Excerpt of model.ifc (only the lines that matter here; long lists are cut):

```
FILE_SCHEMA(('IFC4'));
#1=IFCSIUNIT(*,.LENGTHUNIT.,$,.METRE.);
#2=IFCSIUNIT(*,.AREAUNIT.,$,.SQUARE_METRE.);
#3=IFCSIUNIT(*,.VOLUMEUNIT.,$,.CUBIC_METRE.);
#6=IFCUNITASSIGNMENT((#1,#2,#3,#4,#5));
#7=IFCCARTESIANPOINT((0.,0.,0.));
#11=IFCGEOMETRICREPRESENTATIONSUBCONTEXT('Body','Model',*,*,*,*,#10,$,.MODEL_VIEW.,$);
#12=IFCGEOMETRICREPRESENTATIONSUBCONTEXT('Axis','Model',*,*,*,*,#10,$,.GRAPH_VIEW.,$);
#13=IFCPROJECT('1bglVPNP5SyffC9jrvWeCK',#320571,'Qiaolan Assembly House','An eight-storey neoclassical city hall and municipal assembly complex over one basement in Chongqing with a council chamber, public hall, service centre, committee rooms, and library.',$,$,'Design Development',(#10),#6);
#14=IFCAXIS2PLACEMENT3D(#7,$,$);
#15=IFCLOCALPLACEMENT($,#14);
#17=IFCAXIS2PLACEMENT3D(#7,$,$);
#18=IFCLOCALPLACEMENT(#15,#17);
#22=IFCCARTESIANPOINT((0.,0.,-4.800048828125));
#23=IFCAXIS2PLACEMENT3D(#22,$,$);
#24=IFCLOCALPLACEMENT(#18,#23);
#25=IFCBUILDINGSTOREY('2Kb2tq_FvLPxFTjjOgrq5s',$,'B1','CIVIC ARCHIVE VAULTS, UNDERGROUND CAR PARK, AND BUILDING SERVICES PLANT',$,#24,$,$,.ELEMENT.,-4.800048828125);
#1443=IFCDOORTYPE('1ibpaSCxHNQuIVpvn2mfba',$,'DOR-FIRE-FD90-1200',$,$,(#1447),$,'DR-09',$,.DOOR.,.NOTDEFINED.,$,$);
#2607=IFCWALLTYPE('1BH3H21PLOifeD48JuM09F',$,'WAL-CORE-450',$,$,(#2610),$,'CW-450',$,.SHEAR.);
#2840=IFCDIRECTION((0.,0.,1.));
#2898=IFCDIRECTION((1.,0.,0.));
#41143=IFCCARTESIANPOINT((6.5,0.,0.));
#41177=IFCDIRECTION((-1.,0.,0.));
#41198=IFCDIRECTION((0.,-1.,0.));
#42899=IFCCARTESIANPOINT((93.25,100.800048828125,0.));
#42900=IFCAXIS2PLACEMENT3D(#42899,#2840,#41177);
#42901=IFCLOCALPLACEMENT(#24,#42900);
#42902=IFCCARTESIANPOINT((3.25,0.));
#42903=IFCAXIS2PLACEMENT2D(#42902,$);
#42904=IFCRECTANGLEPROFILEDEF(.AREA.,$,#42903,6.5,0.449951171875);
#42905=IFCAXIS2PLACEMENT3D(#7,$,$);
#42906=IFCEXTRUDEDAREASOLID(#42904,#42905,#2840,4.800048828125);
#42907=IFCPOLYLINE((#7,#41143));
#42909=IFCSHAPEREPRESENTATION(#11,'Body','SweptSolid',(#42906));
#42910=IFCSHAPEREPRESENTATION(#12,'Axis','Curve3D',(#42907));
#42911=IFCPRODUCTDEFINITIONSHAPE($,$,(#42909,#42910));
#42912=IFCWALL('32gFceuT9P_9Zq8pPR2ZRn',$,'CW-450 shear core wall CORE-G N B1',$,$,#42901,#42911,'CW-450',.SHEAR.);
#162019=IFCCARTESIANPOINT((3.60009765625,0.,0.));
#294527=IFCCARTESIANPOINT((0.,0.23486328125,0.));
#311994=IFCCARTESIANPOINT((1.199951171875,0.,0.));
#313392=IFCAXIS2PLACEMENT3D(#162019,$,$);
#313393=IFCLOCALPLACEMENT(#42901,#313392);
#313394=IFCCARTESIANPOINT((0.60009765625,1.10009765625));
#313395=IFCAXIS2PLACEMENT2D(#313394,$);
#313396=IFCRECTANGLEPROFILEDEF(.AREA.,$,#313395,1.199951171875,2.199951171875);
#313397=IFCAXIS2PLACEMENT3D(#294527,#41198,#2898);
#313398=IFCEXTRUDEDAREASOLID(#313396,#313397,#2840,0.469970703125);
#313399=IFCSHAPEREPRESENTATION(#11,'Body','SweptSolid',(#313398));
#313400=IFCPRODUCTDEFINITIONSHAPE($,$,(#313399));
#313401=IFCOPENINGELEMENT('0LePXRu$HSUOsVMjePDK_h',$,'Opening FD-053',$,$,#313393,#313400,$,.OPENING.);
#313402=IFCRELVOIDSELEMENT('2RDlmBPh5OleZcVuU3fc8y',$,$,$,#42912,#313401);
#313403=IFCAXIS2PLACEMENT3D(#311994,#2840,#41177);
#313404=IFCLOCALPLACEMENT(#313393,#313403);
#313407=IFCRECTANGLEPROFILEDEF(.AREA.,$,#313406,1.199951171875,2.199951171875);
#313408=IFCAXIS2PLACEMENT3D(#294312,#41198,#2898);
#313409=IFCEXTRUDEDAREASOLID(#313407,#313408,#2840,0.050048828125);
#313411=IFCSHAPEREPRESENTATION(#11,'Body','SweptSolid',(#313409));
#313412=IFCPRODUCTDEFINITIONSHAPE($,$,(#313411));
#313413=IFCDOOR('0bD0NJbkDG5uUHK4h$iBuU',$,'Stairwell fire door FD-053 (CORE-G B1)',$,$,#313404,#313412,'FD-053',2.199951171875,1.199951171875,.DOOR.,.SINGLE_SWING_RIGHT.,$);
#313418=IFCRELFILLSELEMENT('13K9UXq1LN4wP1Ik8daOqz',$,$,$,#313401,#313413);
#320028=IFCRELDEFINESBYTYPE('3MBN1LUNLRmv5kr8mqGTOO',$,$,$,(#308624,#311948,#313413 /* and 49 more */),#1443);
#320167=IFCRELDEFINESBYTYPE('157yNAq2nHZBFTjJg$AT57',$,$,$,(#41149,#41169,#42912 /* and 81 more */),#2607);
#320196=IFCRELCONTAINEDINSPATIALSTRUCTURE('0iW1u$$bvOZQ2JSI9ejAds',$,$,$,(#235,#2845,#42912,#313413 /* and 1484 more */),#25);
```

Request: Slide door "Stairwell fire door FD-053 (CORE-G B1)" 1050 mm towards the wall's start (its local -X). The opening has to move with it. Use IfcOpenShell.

```python
import ifcopenshell
import ifcopenshell.api.geometry
import ifcopenshell.util.placement

model = ifcopenshell.open("model.ifc")

door = model.by_guid("0bD0NJbkDG5uUHK4h$iBuU")
opening = door.FillsVoids[0].RelatingOpeningElement
wall = opening.VoidsElements[0].RelatingBuildingElement

wall_matrix = ifcopenshell.util.placement.get_local_placement(wall.ObjectPlacement)
shift = wall_matrix[:3, 0] * -1.05
before = ifcopenshell.util.placement.get_local_placement(door.ObjectPlacement)[:3, 3].copy()

# The door is placed relative to its opening, so it follows when the opening moves.
matrix = ifcopenshell.util.placement.get_local_placement(opening.ObjectPlacement)
matrix[:3, 3] += shift
ifcopenshell.api.geometry.edit_object_placement(
    model, product=opening, matrix=matrix, is_si=False, should_transform_children=True
)

after = ifcopenshell.util.placement.get_local_placement(door.ObjectPlacement)[:3, 3]
print("door moved by", (after - before).round(3) + 0.0)

model.write("model_v2.ifc")
```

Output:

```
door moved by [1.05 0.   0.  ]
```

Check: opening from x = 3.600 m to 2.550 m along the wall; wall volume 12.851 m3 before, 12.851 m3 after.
